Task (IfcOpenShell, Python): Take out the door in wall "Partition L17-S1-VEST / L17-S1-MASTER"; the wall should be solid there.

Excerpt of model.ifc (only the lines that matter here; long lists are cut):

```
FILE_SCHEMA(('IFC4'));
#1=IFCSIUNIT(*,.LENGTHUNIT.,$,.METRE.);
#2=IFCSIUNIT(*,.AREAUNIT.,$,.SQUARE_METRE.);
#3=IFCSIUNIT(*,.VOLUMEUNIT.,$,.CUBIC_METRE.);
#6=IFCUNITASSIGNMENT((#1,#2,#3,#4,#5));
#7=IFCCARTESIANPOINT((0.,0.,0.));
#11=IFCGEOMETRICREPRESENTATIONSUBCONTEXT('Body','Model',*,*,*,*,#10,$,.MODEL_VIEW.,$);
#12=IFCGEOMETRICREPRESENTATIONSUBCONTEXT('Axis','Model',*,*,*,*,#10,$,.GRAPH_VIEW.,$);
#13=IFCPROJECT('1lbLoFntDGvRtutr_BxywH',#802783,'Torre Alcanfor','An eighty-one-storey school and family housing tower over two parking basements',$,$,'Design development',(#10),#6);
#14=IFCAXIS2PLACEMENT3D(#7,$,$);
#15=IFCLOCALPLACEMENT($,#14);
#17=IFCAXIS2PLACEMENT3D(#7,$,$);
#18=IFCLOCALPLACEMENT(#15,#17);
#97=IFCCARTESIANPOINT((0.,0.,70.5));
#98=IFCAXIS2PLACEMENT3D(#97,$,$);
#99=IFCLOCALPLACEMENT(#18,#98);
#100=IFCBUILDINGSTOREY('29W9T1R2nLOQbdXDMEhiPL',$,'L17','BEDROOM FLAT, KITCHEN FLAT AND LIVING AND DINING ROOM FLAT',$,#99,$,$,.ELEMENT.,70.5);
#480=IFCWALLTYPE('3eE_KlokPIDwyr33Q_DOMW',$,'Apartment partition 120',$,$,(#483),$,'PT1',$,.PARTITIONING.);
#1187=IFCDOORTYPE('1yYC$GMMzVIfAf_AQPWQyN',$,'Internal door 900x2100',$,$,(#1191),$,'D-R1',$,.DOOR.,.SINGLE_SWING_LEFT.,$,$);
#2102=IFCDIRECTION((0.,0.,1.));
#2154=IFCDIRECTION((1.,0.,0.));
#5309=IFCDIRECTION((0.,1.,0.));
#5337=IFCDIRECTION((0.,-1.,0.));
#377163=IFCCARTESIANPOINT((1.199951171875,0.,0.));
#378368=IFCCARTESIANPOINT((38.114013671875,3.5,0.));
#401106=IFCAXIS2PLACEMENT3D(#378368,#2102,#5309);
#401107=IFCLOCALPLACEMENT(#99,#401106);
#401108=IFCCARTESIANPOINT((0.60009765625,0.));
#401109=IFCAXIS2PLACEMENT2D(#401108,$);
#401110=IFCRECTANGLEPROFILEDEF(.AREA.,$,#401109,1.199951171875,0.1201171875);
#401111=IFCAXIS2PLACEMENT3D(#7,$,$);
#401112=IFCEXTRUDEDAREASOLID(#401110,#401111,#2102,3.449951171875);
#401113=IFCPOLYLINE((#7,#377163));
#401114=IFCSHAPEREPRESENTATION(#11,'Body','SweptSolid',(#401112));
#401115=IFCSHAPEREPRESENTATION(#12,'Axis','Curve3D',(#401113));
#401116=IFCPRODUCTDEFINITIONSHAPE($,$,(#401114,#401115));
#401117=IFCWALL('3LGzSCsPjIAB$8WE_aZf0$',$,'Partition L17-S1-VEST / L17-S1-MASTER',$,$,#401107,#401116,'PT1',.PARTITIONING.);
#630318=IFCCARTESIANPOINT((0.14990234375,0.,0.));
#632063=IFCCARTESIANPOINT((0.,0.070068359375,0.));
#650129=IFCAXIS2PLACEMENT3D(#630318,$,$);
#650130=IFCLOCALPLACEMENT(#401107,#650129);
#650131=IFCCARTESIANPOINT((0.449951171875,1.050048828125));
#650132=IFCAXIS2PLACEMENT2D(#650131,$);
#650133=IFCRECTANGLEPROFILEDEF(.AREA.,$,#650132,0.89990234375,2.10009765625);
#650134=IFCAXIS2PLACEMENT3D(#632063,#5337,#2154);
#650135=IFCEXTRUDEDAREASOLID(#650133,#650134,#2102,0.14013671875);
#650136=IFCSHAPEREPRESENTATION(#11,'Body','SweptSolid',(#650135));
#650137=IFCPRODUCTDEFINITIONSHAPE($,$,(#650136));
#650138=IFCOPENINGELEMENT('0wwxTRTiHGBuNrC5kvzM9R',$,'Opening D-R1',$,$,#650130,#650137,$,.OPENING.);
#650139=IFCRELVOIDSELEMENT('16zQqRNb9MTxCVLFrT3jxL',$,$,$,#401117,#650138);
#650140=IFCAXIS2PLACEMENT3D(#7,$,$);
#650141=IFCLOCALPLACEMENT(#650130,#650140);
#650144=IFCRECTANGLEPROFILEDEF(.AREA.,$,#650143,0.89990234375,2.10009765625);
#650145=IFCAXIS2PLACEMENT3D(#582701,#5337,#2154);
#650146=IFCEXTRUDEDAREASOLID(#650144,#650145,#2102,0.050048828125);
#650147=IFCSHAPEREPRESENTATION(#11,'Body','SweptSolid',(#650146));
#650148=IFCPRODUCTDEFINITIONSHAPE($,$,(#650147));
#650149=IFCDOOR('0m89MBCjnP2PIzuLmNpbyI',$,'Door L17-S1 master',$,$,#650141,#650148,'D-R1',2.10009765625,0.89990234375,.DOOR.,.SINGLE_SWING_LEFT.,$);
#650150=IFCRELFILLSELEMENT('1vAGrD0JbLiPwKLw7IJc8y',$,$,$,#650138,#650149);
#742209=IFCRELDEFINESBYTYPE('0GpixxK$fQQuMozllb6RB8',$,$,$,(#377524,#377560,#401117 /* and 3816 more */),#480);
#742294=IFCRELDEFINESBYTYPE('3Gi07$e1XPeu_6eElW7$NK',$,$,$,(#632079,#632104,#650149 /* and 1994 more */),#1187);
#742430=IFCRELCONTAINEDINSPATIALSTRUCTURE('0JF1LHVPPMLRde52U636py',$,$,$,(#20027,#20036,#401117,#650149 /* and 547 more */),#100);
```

```python
import ifcopenshell
import ifcopenshell.api.feature
import ifcopenshell.api.root
import ifcopenshell.geom
import ifcopenshell.util.shape

model = ifcopenshell.open("model.ifc")
settings = ifcopenshell.geom.settings()


def volume(element):
    """Net volume in cubic metres, openings subtracted."""
    shape = ifcopenshell.geom.create_shape(settings, element)
    return ifcopenshell.util.shape.get_volume(shape.geometry)


door = model.by_guid("0m89MBCjnP2PIzuLmNpbyI")
opening = door.FillsVoids[0].RelatingOpeningElement
wall = opening.VoidsElements[0].RelatingBuildingElement
before = volume(wall)

ifcopenshell.api.root.remove_product(model, product=door)
ifcopenshell.api.feature.remove_feature(model, feature=opening)

after = volume(wall)

print(f"wall volume {before:.3f} -> {after:.3f} m3")

model.write("model_updated.ifc")
```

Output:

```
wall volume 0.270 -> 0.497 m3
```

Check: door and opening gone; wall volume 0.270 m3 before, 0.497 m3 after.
